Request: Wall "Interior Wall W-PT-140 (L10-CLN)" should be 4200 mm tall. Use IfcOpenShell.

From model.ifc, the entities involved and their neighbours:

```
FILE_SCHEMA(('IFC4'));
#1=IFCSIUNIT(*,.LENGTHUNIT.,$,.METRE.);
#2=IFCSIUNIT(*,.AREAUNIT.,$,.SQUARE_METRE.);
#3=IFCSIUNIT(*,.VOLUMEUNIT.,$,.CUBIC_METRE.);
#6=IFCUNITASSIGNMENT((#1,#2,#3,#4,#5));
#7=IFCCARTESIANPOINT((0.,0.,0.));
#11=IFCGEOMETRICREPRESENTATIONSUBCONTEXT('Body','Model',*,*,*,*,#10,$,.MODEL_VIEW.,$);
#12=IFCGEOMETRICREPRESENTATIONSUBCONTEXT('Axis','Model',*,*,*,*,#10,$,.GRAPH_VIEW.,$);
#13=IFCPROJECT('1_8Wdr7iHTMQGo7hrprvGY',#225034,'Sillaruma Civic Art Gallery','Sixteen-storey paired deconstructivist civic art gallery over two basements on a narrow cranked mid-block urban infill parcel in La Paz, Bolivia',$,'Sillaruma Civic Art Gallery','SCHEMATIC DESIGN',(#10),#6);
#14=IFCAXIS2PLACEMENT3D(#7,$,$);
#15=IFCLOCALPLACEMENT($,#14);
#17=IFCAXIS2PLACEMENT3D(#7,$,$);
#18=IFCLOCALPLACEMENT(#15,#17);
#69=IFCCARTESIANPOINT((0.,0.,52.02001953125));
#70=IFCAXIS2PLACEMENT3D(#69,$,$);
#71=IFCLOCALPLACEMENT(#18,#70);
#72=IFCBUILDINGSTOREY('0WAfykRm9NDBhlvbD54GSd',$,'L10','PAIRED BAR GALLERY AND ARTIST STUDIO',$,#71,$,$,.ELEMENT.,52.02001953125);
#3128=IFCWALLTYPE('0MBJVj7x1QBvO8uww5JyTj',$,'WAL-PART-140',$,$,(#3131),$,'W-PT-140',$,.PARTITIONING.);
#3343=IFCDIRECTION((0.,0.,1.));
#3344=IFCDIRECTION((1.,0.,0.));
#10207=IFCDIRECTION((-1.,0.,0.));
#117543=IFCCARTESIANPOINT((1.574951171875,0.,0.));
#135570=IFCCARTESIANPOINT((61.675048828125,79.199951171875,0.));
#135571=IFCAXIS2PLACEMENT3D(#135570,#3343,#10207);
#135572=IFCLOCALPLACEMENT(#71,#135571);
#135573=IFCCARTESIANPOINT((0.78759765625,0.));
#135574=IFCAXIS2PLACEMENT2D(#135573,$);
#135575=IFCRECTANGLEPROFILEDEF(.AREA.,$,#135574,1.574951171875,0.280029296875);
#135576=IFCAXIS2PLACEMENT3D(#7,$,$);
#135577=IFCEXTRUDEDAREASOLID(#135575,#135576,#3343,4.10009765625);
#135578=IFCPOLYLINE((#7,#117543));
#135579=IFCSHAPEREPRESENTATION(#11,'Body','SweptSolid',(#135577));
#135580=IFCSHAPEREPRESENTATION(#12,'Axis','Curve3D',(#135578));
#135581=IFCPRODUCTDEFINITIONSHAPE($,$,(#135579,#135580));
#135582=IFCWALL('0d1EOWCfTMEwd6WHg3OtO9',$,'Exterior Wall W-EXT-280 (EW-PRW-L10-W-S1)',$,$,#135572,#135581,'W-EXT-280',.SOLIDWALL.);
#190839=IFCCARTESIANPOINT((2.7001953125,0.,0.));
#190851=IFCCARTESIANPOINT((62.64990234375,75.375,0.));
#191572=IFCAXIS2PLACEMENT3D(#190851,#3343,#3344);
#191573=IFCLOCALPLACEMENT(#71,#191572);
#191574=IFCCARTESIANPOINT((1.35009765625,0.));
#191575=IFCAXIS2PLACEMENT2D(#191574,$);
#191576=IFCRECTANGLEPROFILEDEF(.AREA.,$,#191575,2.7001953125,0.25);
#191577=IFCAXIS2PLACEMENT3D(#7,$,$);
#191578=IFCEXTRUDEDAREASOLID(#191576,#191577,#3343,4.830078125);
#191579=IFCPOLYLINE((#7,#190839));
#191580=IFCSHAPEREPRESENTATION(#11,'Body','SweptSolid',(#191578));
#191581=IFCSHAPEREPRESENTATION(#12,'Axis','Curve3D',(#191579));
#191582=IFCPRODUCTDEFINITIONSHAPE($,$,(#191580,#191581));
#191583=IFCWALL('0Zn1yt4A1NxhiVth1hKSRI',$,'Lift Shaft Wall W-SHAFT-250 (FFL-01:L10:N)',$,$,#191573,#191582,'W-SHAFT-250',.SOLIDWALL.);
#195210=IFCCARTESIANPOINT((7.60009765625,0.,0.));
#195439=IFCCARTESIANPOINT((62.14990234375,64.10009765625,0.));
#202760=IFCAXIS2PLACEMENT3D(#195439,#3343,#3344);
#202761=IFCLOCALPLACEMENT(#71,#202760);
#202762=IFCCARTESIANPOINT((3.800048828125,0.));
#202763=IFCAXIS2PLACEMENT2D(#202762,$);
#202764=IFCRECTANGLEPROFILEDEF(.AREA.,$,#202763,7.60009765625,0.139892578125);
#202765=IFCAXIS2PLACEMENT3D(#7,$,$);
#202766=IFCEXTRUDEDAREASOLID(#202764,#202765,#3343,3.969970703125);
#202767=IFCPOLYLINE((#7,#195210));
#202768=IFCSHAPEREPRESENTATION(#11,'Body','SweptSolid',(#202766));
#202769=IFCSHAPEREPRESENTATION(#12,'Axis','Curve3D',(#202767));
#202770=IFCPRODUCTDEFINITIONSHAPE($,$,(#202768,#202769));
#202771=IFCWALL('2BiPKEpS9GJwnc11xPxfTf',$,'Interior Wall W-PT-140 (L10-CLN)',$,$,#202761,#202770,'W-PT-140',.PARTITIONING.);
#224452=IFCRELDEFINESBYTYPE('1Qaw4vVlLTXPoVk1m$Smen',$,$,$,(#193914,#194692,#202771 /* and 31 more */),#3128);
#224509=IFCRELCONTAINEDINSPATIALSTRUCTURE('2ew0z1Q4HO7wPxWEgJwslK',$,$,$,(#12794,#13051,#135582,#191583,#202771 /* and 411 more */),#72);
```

```python
import ifcopenshell
import ifcopenshell.geom
import ifcopenshell.util.representation
import ifcopenshell.util.shape
import ifcopenshell.util.unit

model = ifcopenshell.open("model.ifc")
unit_scale = ifcopenshell.util.unit.calculate_unit_scale(model)
settings = ifcopenshell.geom.settings()


def volume(element):
    """Net volume in cubic metres, openings subtracted."""
    shape = ifcopenshell.geom.create_shape(settings, element)
    return ifcopenshell.util.shape.get_volume(shape.geometry)


wall = model.by_guid("2BiPKEpS9GJwnc11xPxfTf")
before = volume(wall)

body = ifcopenshell.util.representation.get_representation(wall, "Model", "Body")
solid = body.Items[0]
old_height = solid.Depth
solid.Depth = 4.2 / unit_scale
after = volume(wall)

print(f"height {old_height:g} -> {solid.Depth:g}, volume {before:.3f} -> {after:.3f} m3")

model.write("model_edited.ifc")
```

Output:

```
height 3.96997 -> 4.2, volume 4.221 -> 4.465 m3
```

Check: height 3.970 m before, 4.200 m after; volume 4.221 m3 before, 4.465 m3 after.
